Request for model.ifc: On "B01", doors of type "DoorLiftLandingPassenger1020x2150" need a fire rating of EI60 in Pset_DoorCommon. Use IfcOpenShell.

First a look at what the model holds.

```python
import ifcopenshell
import ifcopenshell.util.element

model = ifcopenshell.open("model.ifc")
print(model.schema)
storey = next(s for s in model.by_type("IfcBuildingStorey") if s.Name == "B01")
doors = [e for e in ifcopenshell.util.element.get_decomposition(storey) if e.is_a("IfcDoor")]
seen = {}
for e in doors:
    element_type = ifcopenshell.util.element.get_type(e)
    key = (element_type.Name if element_type != e and element_type else None, ifcopenshell.util.element.get_pset(e, "Pset_DoorCommon", "FireRating"))
    seen[key] = seen.get(key, 0) + 1
for (name, value), count in sorted(seen.items(), key=str):
    print(count, "x", name, "|", value)
```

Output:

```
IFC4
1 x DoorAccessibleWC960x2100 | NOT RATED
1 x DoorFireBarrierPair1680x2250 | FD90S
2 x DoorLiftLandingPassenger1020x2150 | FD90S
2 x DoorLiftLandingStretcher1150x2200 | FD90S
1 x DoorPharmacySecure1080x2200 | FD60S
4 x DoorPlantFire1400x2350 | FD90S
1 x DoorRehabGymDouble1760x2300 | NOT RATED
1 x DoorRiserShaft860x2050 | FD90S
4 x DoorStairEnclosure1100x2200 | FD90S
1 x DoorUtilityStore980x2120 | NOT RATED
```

```python
import ifcopenshell
import ifcopenshell.api.pset
import ifcopenshell.util.element

model = ifcopenshell.open("model.ifc")

storey = next(s for s in model.by_type("IfcBuildingStorey") if s.Name == "B01")
doors = [e for e in ifcopenshell.util.element.get_decomposition(storey) if e.is_a("IfcDoor")]

count = 0
for e in doors:
    element_type = ifcopenshell.util.element.get_type(e)
    if element_type in (None, e) or element_type.Name != "DoorLiftLandingPassenger1020x2150":
        continue
    # add_pset returns the element's existing set when there is one.
    pset = ifcopenshell.api.pset.add_pset(model, product=e, name="Pset_DoorCommon")
    ifcopenshell.api.pset.edit_pset(model, pset=pset, properties={"FireRating": "EI60"})
    count += 1

print(count, "doors updated")

model.write("model-out.ifc")
```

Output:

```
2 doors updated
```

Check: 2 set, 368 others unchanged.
